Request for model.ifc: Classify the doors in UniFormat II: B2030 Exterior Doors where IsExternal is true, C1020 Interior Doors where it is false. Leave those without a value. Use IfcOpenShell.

First a look at what the model holds.

```python
import ifcopenshell
import ifcopenshell.util.element

model = ifcopenshell.open("model.ifc")
print(model.schema)
print("classifications:", [c.Name for c in model.by_type("IfcClassification")])
values = [ifcopenshell.util.element.get_pset(e, "Pset_DoorCommon", "IsExternal") for e in model.by_type("IfcDoor")]
for value in (True, False, None):
    print("IsExternal", value, values.count(value))
```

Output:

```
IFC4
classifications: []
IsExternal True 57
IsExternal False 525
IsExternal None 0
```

```python
import ifcopenshell
import ifcopenshell.api.classification
import ifcopenshell.util.element

model = ifcopenshell.open("model.ifc")

system = ifcopenshell.api.classification.add_classification(model, classification="UniFormat II")

doors = model.by_type("IfcDoor")
external = {e: ifcopenshell.util.element.get_pset(e, "Pset_DoorCommon", "IsExternal") for e in doors}
for flag, code, name in ((True, "B2030", "Exterior Doors"), (False, "C1020", "Interior Doors")):
    products = [e for e in doors if external[e] is flag]
    ifcopenshell.api.classification.add_reference(
        model, products=products, classification=system, identification=code, name=name
    )
    print(code, len(products))

model.write("model-out.ifc")
```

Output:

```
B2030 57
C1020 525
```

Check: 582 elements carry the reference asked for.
